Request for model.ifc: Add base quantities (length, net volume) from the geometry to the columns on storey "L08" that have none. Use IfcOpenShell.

First a look at what the model holds.

```python
import ifcopenshell
import ifcopenshell.util.element
import ifcopenshell.util.unit

model = ifcopenshell.open("model.ifc")
print(model.schema)
for unit_type in ("LENGTHUNIT", "AREAUNIT", "VOLUMEUNIT"):
    print(unit_type, ifcopenshell.util.unit.calculate_unit_scale(model, unit_type))
storey = next(s for s in model.by_type("IfcBuildingStorey") if s.Name == "L08")
columns = [e for e in ifcopenshell.util.element.get_decomposition(storey) if e.is_a("IfcColumn")]
for e in sorted(columns, key=lambda e: e.id()):
    print(e.id(), e.is_a(), e.Name, list(ifcopenshell.util.element.get_psets(e, qtos_only=True)), sep=" | ")
```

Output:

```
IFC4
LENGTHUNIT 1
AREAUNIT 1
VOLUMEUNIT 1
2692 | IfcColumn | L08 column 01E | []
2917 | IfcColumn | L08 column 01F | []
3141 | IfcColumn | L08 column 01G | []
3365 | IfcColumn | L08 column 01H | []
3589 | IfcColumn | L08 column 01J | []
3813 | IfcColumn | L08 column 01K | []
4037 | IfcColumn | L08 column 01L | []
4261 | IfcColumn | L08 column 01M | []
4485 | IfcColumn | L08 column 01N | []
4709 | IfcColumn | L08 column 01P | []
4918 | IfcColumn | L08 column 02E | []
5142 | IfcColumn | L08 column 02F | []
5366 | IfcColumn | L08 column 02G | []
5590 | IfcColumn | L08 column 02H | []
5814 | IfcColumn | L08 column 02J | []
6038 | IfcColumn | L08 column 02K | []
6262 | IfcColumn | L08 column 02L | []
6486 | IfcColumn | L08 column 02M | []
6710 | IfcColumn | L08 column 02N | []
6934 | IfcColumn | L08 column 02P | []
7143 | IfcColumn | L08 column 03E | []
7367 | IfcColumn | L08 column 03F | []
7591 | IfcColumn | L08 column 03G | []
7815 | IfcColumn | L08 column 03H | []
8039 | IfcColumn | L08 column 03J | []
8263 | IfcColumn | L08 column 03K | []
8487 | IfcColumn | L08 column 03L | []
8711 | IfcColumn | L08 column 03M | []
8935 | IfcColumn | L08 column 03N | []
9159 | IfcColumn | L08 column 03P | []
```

```python
import ifcopenshell
import ifcopenshell.api.pset
import ifcopenshell.geom
import ifcopenshell.util.element
import ifcopenshell.util.shape
import ifcopenshell.util.unit

model = ifcopenshell.open("model.ifc")
unit_scale = ifcopenshell.util.unit.calculate_unit_scale(model)
volume_scale = ifcopenshell.util.unit.calculate_unit_scale(model, "VOLUMEUNIT")
settings = ifcopenshell.geom.settings()

storey = next(s for s in model.by_type("IfcBuildingStorey") if s.Name == "L08")
columns = [e for e in ifcopenshell.util.element.get_decomposition(storey) if e.is_a("IfcColumn")]

for e in sorted(columns, key=lambda e: e.id()):
    if ifcopenshell.util.element.get_psets(e, qtos_only=True, should_inherit=False):
        continue
    # Geometry comes back in metres, in the element's own axes.
    shape = ifcopenshell.geom.create_shape(settings, e)
    values = {
        "Length": ifcopenshell.util.shape.get_z(shape.geometry) / unit_scale,
        "NetVolume": ifcopenshell.util.shape.get_volume(shape.geometry) / volume_scale,
    }
    qto = ifcopenshell.api.pset.add_qto(model, product=e, name="Qto_ColumnBaseQuantities")
    ifcopenshell.api.pset.edit_qto(model, qto=qto, properties=values)
    print(e.id(), {k: round(v, 3) for k, v in values.items()})

model.write("model-out.ifc")
```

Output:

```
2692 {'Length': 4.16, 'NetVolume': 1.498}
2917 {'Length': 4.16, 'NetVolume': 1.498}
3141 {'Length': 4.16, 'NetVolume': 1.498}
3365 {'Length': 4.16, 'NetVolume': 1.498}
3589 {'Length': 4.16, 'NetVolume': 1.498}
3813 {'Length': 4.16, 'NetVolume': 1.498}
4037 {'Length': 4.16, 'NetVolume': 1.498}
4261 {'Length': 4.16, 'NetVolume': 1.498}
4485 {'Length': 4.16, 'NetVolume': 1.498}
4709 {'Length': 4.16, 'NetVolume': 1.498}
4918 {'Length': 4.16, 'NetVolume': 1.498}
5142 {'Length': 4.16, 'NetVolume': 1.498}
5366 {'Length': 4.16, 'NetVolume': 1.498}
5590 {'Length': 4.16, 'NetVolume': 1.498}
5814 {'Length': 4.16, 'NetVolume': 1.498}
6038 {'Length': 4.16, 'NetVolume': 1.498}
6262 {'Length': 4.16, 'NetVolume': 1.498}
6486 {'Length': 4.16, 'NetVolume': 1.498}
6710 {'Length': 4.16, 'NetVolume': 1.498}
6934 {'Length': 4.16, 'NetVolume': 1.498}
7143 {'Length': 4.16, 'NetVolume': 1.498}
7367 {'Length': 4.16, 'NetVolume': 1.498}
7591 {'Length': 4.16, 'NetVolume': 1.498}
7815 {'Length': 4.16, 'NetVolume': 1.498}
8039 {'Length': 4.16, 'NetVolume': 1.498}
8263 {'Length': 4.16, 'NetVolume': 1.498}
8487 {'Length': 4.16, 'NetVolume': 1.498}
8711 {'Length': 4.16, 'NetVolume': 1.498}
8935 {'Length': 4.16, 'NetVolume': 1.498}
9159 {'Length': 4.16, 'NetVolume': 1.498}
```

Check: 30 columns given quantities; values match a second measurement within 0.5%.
